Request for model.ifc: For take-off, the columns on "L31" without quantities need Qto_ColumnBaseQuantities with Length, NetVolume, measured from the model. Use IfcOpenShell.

First a look at what the model holds.

```python
import ifcopenshell
import ifcopenshell.util.element
import ifcopenshell.util.unit

model = ifcopenshell.open("model.ifc")
print(model.schema)
for unit_type in ("LENGTHUNIT", "AREAUNIT", "VOLUMEUNIT"):
    print(unit_type, ifcopenshell.util.unit.calculate_unit_scale(model, unit_type))
storey = next(s for s in model.by_type("IfcBuildingStorey") if s.Name == "L31")
columns = [e for e in ifcopenshell.util.element.get_decomposition(storey) if e.is_a("IfcColumn")]
for e in sorted(columns, key=lambda e: e.id()):
    print(e.id(), e.is_a(), e.Name, list(ifcopenshell.util.element.get_psets(e, qtos_only=True)), sep=" | ")
```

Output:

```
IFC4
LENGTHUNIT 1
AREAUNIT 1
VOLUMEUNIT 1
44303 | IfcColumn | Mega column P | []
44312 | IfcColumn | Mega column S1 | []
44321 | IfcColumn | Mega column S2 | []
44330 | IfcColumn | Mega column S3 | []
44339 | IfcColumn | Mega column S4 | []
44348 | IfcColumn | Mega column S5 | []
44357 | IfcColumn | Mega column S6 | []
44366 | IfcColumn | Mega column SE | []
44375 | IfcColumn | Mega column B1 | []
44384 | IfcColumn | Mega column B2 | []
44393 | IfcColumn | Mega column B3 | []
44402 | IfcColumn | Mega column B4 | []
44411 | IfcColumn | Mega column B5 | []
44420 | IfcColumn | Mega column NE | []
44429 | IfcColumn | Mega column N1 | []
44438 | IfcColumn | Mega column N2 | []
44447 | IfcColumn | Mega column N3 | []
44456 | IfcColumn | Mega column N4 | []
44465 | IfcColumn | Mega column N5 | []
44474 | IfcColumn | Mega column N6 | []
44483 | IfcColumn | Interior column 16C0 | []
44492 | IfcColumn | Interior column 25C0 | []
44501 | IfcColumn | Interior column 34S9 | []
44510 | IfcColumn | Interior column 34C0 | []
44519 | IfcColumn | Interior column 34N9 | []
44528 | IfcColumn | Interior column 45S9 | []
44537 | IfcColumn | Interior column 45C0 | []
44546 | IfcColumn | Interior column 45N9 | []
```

```python
import ifcopenshell
import ifcopenshell.api.pset
import ifcopenshell.geom
import ifcopenshell.util.element
import ifcopenshell.util.shape
import ifcopenshell.util.unit

model = ifcopenshell.open("model.ifc")
unit_scale = ifcopenshell.util.unit.calculate_unit_scale(model)
volume_scale = ifcopenshell.util.unit.calculate_unit_scale(model, "VOLUMEUNIT")
settings = ifcopenshell.geom.settings()

storey = next(s for s in model.by_type("IfcBuildingStorey") if s.Name == "L31")
columns = [e for e in ifcopenshell.util.element.get_decomposition(storey) if e.is_a("IfcColumn")]

for e in sorted(columns, key=lambda e: e.id()):
    if ifcopenshell.util.element.get_psets(e, qtos_only=True, should_inherit=False):
        continue
    # Geometry comes back in metres, in the element's own axes.
    shape = ifcopenshell.geom.create_shape(settings, e)
    values = {
        "Length": ifcopenshell.util.shape.get_z(shape.geometry) / unit_scale,
        "NetVolume": ifcopenshell.util.shape.get_volume(shape.geometry) / volume_scale,
    }
    qto = ifcopenshell.api.pset.add_qto(model, product=e, name="Qto_ColumnBaseQuantities")
    ifcopenshell.api.pset.edit_qto(model, qto=qto, properties=values)
    print(e.id(), {k: round(v, 3) for k, v in values.items()})

model.write("model_v2.ifc")
```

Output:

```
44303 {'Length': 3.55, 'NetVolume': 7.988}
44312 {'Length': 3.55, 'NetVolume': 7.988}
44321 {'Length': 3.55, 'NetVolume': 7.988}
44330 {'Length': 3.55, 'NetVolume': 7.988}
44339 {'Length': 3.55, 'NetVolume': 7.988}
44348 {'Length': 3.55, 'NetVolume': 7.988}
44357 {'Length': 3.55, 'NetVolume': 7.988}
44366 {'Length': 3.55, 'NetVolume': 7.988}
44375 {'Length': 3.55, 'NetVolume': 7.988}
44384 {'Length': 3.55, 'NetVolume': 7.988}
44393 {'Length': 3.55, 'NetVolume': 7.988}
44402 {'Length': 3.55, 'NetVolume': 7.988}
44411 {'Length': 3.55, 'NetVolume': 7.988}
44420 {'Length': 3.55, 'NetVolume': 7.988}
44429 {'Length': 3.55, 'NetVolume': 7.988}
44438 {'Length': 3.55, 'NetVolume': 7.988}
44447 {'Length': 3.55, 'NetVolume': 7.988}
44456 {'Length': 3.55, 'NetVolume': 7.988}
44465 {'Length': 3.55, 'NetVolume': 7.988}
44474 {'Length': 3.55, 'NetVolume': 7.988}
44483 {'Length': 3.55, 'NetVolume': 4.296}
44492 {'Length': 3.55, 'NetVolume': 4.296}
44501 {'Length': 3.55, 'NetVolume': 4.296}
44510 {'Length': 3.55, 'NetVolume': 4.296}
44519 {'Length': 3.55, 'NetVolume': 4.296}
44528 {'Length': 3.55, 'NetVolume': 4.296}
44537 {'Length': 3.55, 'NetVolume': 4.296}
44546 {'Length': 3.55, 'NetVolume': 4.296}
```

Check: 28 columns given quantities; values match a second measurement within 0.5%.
